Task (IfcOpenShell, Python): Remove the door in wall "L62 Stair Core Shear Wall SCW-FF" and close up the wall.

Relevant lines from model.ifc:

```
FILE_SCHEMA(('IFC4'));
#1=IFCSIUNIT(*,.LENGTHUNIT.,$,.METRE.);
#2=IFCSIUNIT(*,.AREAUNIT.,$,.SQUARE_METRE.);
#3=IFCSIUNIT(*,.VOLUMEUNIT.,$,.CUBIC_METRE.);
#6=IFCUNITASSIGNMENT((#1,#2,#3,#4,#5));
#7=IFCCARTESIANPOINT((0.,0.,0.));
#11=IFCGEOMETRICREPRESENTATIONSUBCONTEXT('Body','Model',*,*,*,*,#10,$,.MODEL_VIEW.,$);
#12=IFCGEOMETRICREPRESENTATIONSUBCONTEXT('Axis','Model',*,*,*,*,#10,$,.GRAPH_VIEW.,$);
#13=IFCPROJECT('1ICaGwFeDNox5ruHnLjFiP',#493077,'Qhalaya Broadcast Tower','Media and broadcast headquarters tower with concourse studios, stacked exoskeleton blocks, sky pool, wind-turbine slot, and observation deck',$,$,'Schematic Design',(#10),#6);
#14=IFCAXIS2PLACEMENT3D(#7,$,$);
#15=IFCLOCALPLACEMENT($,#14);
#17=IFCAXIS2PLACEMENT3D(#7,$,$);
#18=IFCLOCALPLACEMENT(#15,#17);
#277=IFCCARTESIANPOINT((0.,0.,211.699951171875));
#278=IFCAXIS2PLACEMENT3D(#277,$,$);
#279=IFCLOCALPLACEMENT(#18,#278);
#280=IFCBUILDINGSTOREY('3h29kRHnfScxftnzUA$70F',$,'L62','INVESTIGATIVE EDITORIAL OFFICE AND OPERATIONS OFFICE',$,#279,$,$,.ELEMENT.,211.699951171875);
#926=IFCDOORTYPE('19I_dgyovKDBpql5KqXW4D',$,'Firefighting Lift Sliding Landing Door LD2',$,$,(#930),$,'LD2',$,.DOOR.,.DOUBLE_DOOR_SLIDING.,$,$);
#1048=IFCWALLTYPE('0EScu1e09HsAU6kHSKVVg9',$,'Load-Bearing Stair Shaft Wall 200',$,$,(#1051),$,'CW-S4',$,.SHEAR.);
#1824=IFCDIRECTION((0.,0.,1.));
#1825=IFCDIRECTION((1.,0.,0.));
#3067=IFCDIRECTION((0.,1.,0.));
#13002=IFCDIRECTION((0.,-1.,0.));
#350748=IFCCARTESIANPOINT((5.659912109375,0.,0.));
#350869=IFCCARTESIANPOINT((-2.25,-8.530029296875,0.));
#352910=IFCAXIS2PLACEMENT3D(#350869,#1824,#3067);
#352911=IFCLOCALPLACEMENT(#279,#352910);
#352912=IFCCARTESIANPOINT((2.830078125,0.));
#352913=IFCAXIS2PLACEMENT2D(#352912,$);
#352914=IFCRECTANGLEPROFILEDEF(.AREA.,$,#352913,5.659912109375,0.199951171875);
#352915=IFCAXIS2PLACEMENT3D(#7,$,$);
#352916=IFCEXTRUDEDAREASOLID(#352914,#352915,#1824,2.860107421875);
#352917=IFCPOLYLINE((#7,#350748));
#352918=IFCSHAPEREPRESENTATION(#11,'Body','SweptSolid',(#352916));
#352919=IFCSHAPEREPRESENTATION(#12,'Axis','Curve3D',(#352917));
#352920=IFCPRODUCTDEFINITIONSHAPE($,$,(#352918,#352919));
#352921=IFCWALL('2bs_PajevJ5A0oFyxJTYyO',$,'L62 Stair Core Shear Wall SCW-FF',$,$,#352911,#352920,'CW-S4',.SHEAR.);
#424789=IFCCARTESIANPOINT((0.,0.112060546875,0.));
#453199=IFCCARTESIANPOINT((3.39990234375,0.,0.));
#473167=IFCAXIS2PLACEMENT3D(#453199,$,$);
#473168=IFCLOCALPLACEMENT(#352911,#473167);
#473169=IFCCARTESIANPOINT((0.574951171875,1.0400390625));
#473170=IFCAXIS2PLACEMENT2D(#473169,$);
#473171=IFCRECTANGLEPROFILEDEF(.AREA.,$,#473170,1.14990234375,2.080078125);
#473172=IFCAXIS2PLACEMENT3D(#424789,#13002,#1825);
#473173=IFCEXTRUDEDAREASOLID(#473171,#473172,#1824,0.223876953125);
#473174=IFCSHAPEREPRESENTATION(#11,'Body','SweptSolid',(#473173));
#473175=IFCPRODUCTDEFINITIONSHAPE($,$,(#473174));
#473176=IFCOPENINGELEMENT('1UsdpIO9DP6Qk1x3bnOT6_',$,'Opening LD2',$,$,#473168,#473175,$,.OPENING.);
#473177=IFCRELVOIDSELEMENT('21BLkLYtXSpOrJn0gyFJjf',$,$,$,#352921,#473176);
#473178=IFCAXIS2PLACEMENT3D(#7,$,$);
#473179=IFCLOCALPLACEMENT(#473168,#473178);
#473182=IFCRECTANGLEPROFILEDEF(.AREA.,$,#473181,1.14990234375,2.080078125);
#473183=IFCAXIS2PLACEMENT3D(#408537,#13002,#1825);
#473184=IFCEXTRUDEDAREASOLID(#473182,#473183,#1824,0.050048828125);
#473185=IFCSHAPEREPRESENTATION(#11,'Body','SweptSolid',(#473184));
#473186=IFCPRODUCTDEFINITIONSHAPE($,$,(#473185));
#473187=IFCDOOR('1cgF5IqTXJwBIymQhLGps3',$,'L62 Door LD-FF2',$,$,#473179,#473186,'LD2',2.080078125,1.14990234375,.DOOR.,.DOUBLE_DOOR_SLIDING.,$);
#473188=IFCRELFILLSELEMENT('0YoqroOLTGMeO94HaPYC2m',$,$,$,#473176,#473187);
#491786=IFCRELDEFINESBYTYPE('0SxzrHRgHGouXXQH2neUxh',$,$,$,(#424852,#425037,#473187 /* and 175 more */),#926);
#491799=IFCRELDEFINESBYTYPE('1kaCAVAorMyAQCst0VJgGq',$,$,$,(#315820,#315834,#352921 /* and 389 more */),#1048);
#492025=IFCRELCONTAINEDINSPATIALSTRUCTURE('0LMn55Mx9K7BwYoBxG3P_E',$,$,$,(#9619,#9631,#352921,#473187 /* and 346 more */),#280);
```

```python
import ifcopenshell
import ifcopenshell.api.feature
import ifcopenshell.api.root
import ifcopenshell.geom
import ifcopenshell.util.shape

model = ifcopenshell.open("model.ifc")
settings = ifcopenshell.geom.settings()


def volume(element):
    """Net volume in cubic metres, openings subtracted."""
    shape = ifcopenshell.geom.create_shape(settings, element)
    return ifcopenshell.util.shape.get_volume(shape.geometry)


door = model.by_guid("1cgF5IqTXJwBIymQhLGps3")
opening = door.FillsVoids[0].RelatingOpeningElement
wall = opening.VoidsElements[0].RelatingBuildingElement
before = volume(wall)

ifcopenshell.api.root.remove_product(model, product=door)
ifcopenshell.api.feature.remove_feature(model, feature=opening)

after = volume(wall)

print(f"wall volume {before:.3f} -> {after:.3f} m3")

model.write("model_updated.ifc")
```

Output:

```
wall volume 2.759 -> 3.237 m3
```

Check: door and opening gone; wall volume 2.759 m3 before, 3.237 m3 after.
